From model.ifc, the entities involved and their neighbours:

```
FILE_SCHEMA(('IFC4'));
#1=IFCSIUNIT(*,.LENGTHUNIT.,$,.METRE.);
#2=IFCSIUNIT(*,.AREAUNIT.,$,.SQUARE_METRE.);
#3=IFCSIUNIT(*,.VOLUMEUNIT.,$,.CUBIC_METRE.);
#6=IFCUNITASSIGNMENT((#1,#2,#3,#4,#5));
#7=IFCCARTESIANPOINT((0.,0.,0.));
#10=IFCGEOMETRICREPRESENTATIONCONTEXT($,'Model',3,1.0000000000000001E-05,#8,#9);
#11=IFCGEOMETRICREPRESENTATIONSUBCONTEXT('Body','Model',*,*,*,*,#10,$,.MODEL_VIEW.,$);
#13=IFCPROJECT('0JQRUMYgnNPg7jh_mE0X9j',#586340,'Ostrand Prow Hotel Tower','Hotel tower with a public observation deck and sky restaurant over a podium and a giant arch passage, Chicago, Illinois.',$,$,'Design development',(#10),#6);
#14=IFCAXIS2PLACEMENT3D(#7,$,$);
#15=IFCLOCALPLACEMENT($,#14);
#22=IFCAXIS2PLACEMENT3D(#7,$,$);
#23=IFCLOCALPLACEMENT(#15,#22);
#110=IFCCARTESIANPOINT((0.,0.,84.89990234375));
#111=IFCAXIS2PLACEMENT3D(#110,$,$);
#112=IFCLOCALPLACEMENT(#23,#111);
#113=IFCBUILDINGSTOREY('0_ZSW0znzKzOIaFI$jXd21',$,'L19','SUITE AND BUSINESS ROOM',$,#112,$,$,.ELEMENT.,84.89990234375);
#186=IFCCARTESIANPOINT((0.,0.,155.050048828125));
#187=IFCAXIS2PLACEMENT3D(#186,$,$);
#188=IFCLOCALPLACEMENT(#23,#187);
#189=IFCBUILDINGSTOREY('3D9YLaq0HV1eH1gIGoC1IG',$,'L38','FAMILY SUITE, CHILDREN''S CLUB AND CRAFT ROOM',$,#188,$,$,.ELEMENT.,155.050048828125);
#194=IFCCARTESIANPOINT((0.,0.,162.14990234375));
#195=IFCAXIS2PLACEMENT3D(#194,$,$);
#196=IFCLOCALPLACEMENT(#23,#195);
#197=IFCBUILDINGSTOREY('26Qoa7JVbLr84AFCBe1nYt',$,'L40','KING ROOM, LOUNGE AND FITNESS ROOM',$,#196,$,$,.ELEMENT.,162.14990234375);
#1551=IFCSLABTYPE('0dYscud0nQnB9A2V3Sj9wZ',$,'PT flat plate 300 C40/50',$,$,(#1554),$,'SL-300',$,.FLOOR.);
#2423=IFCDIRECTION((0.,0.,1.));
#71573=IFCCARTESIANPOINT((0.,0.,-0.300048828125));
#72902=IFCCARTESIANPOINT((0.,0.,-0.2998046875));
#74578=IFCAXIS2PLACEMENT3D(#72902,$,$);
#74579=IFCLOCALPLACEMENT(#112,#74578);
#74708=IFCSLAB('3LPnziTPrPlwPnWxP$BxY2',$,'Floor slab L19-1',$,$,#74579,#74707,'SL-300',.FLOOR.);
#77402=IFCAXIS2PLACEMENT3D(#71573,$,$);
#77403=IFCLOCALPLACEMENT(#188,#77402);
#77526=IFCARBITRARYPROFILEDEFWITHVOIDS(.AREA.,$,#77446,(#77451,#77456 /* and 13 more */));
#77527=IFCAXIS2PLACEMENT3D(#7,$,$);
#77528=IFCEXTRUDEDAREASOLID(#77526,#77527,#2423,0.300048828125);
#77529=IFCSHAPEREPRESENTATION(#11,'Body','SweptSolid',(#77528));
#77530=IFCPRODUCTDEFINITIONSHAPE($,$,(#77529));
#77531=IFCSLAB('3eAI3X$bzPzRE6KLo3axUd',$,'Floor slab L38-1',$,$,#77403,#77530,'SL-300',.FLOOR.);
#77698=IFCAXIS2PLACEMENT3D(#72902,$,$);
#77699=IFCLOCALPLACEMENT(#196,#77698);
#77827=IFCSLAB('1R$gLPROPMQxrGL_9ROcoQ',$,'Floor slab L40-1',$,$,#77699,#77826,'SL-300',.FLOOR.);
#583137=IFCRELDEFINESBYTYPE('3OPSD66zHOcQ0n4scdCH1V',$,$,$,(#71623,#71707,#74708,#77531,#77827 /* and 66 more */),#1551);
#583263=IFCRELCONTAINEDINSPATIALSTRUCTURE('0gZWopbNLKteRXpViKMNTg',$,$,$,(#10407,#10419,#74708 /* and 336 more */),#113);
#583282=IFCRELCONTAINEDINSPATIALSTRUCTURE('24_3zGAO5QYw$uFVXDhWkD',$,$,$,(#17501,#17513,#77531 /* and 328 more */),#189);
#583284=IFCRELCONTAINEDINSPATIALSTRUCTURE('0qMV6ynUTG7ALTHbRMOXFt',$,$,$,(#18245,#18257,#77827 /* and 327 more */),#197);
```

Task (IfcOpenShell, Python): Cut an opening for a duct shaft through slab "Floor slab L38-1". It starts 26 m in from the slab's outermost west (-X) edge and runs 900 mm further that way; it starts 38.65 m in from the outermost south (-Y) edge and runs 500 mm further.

```python
import numpy as np
import ifcopenshell
import ifcopenshell.api.feature
import ifcopenshell.api.geometry
import ifcopenshell.api.root
import ifcopenshell.geom
import ifcopenshell.util.placement
import ifcopenshell.util.representation
import ifcopenshell.util.shape
import ifcopenshell.util.unit

model = ifcopenshell.open("model.ifc")
unit_scale = ifcopenshell.util.unit.calculate_unit_scale(model)
settings = ifcopenshell.geom.settings()


def volume(element):
    """Net volume in cubic metres, openings subtracted."""
    shape = ifcopenshell.geom.create_shape(settings, element)
    return ifcopenshell.util.shape.get_volume(shape.geometry)


slab = model.by_id(77531)
before = volume(slab)

# Extent in the slab's own axes, in metres. The edges named are its -X and -Y sides.
slab_shape = ifcopenshell.geom.create_shape(settings, slab)
vertices = ifcopenshell.util.shape.get_vertices(slab_shape.geometry)
x_min, y_min, bottom = vertices.min(axis=0)
top = vertices[:, 2].max()

opening = ifcopenshell.api.root.create_entity(model, ifc_class="IfcOpeningElement", name="Duct shaft opening", predefined_type="OPENING")
context = ifcopenshell.util.representation.get_context(model, "Model", "Body", "MODEL_VIEW")
width, depth = 0.9, 0.5
outline = [(0.0, 0.0), (width, 0.0), (width, depth), (0.0, depth), (0.0, 0.0)]
# Overshoot both faces by 50 mm so the cut is clean.
shape = ifcopenshell.api.geometry.add_slab_representation(
    model, context=context, depth=top - bottom + 0.1, polyline=outline
)
ifcopenshell.api.geometry.assign_representation(model, product=opening, representation=shape)

matrix = ifcopenshell.util.placement.get_local_placement(slab.ObjectPlacement)
matrix[:, 3] = matrix @ np.append(np.array([x_min + 26, y_min + 38.65, bottom - 0.05]) / unit_scale, 1.0)
ifcopenshell.api.geometry.edit_object_placement(model, product=opening, matrix=matrix, is_si=False)
ifcopenshell.api.feature.add_feature(model, feature=opening, element=slab)

after = volume(slab)

print(f"slab volume {before:.3f} -> {after:.3f} m3")

model.write("model_updated.ifc")
```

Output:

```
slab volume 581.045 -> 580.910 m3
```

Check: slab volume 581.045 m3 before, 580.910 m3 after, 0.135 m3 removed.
